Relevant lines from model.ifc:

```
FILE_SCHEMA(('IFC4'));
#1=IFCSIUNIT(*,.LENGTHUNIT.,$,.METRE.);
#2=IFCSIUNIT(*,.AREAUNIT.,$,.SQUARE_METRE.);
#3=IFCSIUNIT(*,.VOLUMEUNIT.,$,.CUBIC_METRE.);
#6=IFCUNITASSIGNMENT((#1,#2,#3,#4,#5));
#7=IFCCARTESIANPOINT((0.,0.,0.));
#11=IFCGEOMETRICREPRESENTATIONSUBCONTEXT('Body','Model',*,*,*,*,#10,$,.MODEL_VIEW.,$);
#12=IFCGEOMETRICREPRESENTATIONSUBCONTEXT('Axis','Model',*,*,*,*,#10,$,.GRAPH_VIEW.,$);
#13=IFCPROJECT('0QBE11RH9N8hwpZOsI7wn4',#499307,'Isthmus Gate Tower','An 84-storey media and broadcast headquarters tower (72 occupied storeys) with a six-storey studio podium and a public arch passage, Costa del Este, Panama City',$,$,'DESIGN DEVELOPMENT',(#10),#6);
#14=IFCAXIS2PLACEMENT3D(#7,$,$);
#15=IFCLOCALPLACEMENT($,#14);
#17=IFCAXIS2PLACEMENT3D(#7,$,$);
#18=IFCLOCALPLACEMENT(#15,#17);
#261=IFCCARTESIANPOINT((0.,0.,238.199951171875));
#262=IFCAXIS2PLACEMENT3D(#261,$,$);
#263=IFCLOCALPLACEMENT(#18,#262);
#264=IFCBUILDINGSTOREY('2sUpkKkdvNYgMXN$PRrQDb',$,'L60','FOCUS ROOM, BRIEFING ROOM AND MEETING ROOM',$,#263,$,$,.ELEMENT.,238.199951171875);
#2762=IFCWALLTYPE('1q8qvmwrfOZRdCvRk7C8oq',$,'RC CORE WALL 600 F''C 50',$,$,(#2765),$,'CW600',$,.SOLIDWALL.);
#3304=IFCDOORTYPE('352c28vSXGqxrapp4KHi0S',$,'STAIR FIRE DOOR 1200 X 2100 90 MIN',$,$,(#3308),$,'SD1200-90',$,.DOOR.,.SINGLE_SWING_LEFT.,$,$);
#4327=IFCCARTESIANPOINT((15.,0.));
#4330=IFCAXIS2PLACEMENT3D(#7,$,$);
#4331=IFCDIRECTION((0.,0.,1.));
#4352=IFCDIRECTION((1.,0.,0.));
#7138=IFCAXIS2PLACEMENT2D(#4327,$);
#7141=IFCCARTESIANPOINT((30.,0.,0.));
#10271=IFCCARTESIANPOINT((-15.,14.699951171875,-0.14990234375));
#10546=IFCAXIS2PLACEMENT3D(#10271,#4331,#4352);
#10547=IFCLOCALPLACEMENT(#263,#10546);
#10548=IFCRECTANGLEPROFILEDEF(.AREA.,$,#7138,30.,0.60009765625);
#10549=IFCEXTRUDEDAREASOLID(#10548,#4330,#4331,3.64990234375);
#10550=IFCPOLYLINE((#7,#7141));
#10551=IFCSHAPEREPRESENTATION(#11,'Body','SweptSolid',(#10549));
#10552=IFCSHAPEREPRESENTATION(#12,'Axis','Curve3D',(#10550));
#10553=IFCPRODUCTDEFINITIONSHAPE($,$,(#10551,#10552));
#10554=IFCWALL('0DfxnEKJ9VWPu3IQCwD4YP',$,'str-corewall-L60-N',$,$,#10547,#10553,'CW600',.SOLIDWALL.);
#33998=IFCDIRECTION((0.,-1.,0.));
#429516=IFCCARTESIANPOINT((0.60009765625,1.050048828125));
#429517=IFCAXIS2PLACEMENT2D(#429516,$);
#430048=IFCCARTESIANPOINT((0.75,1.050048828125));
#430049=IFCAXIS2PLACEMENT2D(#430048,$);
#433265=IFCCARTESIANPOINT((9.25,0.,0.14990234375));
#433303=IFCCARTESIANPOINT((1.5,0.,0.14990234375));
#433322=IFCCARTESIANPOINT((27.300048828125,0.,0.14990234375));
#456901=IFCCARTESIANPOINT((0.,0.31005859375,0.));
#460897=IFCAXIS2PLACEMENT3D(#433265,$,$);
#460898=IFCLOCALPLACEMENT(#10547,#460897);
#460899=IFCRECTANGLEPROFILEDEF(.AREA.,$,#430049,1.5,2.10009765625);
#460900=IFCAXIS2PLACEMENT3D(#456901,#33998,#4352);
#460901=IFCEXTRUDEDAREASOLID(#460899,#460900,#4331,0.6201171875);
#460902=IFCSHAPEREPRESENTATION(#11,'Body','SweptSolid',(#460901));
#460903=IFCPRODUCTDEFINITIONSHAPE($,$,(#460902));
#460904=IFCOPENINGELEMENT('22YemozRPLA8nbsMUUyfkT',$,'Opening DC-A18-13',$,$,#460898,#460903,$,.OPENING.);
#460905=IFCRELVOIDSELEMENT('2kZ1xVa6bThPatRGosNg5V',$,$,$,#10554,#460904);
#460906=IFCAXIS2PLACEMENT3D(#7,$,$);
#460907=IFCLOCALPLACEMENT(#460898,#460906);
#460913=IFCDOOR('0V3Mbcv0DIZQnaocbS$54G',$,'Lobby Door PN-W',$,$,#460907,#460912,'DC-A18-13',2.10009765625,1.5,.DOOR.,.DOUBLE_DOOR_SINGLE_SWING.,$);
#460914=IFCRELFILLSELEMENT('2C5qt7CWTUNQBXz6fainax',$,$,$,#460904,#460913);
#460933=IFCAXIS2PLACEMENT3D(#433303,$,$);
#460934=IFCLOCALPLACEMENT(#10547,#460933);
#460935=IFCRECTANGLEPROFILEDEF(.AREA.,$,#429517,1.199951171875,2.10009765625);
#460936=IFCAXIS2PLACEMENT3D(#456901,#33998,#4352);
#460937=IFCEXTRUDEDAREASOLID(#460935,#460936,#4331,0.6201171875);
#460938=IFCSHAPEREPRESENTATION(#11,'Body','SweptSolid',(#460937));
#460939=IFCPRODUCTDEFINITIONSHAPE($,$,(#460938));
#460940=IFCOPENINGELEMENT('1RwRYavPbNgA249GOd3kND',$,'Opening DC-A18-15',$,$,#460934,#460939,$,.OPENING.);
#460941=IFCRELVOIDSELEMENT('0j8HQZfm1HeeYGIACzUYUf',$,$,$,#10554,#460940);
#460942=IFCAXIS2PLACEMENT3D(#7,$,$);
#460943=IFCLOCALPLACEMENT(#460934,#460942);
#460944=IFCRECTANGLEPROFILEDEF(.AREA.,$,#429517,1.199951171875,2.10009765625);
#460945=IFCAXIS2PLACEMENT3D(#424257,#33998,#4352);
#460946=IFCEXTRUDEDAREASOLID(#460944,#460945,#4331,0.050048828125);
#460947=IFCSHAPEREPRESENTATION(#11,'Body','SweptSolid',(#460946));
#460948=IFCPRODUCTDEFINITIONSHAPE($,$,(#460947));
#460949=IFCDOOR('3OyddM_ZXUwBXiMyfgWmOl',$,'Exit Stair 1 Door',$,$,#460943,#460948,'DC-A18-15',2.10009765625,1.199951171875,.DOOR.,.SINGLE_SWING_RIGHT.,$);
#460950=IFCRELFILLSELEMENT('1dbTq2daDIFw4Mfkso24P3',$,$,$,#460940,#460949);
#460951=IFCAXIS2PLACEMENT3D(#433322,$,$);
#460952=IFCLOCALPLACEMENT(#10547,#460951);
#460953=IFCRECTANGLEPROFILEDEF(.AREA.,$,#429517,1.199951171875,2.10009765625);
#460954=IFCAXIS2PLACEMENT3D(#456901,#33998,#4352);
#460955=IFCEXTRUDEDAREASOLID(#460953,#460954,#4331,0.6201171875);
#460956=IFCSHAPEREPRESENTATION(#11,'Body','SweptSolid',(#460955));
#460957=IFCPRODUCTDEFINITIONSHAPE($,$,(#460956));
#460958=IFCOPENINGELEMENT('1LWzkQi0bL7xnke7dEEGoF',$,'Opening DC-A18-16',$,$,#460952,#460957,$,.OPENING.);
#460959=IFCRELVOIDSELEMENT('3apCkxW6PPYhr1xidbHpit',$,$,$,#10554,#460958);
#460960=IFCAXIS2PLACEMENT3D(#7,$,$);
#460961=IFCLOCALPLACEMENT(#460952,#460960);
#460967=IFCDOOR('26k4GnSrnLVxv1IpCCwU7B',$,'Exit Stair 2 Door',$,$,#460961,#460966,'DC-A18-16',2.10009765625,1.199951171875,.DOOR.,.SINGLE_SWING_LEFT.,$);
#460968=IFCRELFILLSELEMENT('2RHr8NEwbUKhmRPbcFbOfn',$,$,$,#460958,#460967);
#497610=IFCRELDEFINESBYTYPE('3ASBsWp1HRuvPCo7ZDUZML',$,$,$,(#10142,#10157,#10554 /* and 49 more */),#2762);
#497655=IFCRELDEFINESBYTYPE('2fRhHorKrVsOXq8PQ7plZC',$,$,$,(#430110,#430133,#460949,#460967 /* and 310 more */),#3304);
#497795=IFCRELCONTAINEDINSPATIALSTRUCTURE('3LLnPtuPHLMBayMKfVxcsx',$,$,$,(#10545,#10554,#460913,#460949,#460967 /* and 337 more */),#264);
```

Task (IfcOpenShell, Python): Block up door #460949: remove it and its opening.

```python
import ifcopenshell
import ifcopenshell.api.feature
import ifcopenshell.api.root
import ifcopenshell.geom
import ifcopenshell.util.shape

model = ifcopenshell.open("model.ifc")
settings = ifcopenshell.geom.settings()


def volume(element):
    """Net volume in cubic metres, openings subtracted."""
    shape = ifcopenshell.geom.create_shape(settings, element)
    return ifcopenshell.util.shape.get_volume(shape.geometry)


door = model.by_guid("3OyddM_ZXUwBXiMyfgWmOl")
opening = door.FillsVoids[0].RelatingOpeningElement
wall = opening.VoidsElements[0].RelatingBuildingElement
before = volume(wall)

ifcopenshell.api.root.remove_product(model, product=door)
ifcopenshell.api.feature.remove_feature(model, feature=opening)

after = volume(wall)

print(f"wall volume {before:.3f} -> {after:.3f} m3")

model.write("model_v2.ifc")
```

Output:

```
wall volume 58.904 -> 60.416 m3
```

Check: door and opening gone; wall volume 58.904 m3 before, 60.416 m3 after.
